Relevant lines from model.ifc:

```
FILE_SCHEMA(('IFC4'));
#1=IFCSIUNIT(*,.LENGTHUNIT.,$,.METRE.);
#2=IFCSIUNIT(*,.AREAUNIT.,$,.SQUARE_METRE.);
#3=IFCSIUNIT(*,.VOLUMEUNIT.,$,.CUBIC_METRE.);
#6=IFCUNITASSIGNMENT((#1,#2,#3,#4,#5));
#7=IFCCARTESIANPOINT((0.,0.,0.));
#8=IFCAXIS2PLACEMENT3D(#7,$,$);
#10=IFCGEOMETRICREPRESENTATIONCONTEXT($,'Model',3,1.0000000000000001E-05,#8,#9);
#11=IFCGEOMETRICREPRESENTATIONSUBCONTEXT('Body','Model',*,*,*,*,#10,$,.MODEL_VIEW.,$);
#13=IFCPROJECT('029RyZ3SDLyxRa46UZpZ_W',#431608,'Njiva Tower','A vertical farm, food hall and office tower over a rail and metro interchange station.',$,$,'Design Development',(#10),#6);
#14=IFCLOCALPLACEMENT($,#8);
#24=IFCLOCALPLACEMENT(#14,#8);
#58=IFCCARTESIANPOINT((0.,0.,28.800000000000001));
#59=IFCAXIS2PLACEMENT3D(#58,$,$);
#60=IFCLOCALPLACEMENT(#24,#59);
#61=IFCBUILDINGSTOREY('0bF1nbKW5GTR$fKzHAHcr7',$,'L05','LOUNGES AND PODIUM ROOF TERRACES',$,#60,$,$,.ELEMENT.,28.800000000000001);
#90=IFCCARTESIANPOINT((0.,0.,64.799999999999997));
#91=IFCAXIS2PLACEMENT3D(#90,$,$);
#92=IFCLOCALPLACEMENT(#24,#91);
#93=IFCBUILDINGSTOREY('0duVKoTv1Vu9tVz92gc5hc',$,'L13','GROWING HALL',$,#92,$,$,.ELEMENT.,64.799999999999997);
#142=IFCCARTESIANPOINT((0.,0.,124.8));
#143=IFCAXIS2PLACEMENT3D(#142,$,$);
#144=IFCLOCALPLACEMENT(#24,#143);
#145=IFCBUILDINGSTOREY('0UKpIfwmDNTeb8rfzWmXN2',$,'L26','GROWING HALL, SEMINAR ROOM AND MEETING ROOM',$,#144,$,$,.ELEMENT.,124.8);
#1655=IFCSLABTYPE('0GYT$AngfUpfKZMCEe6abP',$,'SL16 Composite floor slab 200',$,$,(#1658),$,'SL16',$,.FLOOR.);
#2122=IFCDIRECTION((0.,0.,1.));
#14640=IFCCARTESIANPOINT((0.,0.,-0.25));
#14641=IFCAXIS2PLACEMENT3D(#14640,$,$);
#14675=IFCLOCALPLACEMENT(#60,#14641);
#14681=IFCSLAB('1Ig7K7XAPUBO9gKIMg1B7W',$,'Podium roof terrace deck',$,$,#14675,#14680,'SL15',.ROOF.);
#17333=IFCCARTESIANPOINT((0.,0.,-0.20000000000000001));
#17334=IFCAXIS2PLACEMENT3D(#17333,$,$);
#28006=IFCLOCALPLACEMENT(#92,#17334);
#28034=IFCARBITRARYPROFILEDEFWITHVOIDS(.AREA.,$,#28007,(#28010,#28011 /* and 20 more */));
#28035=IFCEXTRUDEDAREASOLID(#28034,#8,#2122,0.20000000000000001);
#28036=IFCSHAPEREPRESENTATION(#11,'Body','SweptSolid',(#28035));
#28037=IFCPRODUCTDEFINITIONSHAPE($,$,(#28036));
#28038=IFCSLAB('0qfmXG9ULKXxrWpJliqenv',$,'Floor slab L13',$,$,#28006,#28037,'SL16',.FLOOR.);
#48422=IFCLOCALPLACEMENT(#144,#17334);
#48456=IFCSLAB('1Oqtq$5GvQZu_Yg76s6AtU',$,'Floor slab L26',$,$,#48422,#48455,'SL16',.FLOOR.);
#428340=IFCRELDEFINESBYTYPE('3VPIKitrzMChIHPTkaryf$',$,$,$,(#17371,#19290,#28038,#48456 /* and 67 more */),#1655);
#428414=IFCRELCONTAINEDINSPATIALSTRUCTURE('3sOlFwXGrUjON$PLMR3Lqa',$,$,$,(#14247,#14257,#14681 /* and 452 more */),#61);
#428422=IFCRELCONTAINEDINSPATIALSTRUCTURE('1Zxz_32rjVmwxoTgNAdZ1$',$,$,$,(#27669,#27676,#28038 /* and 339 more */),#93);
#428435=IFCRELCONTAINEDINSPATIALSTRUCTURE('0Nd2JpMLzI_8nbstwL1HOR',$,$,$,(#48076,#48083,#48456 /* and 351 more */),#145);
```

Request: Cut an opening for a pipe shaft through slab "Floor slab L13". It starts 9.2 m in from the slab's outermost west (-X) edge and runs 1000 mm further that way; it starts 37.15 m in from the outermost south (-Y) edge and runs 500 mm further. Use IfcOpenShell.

```python
import numpy as np
import ifcopenshell
import ifcopenshell.api.feature
import ifcopenshell.api.geometry
import ifcopenshell.api.root
import ifcopenshell.geom
import ifcopenshell.util.placement
import ifcopenshell.util.representation
import ifcopenshell.util.shape
import ifcopenshell.util.unit

model = ifcopenshell.open("model.ifc")
unit_scale = ifcopenshell.util.unit.calculate_unit_scale(model)
settings = ifcopenshell.geom.settings()


def volume(element):
    """Net volume in cubic metres, openings subtracted."""
    shape = ifcopenshell.geom.create_shape(settings, element)
    return ifcopenshell.util.shape.get_volume(shape.geometry)


slab = model.by_guid("0qfmXG9ULKXxrWpJliqenv")
before = volume(slab)

# Extent in the slab's own axes, in metres. The edges named are its -X and -Y sides.
slab_shape = ifcopenshell.geom.create_shape(settings, slab)
vertices = ifcopenshell.util.shape.get_vertices(slab_shape.geometry)
x_min, y_min, bottom = vertices.min(axis=0)
top = vertices[:, 2].max()

opening = ifcopenshell.api.root.create_entity(model, ifc_class="IfcOpeningElement", name="Pipe shaft opening", predefined_type="OPENING")
context = ifcopenshell.util.representation.get_context(model, "Model", "Body", "MODEL_VIEW")
width, depth = 1, 0.5
outline = [(0.0, 0.0), (width, 0.0), (width, depth), (0.0, depth), (0.0, 0.0)]
# Overshoot both faces by 50 mm so the cut is clean.
shape = ifcopenshell.api.geometry.add_slab_representation(
    model, context=context, depth=top - bottom + 0.1, polyline=outline
)
ifcopenshell.api.geometry.assign_representation(model, product=opening, representation=shape)

matrix = ifcopenshell.util.placement.get_local_placement(slab.ObjectPlacement)
matrix[:, 3] = matrix @ np.append(np.array([x_min + 9.2, y_min + 37.15, bottom - 0.05]) / unit_scale, 1.0)
ifcopenshell.api.geometry.edit_object_placement(model, product=opening, matrix=matrix, is_si=False)
ifcopenshell.api.feature.add_feature(model, feature=opening, element=slab)

after = volume(slab)

print(f"slab volume {before:.3f} -> {after:.3f} m3")

model.write("model_edited.ifc")
```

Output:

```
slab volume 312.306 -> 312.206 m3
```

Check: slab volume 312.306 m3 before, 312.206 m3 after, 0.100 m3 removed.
